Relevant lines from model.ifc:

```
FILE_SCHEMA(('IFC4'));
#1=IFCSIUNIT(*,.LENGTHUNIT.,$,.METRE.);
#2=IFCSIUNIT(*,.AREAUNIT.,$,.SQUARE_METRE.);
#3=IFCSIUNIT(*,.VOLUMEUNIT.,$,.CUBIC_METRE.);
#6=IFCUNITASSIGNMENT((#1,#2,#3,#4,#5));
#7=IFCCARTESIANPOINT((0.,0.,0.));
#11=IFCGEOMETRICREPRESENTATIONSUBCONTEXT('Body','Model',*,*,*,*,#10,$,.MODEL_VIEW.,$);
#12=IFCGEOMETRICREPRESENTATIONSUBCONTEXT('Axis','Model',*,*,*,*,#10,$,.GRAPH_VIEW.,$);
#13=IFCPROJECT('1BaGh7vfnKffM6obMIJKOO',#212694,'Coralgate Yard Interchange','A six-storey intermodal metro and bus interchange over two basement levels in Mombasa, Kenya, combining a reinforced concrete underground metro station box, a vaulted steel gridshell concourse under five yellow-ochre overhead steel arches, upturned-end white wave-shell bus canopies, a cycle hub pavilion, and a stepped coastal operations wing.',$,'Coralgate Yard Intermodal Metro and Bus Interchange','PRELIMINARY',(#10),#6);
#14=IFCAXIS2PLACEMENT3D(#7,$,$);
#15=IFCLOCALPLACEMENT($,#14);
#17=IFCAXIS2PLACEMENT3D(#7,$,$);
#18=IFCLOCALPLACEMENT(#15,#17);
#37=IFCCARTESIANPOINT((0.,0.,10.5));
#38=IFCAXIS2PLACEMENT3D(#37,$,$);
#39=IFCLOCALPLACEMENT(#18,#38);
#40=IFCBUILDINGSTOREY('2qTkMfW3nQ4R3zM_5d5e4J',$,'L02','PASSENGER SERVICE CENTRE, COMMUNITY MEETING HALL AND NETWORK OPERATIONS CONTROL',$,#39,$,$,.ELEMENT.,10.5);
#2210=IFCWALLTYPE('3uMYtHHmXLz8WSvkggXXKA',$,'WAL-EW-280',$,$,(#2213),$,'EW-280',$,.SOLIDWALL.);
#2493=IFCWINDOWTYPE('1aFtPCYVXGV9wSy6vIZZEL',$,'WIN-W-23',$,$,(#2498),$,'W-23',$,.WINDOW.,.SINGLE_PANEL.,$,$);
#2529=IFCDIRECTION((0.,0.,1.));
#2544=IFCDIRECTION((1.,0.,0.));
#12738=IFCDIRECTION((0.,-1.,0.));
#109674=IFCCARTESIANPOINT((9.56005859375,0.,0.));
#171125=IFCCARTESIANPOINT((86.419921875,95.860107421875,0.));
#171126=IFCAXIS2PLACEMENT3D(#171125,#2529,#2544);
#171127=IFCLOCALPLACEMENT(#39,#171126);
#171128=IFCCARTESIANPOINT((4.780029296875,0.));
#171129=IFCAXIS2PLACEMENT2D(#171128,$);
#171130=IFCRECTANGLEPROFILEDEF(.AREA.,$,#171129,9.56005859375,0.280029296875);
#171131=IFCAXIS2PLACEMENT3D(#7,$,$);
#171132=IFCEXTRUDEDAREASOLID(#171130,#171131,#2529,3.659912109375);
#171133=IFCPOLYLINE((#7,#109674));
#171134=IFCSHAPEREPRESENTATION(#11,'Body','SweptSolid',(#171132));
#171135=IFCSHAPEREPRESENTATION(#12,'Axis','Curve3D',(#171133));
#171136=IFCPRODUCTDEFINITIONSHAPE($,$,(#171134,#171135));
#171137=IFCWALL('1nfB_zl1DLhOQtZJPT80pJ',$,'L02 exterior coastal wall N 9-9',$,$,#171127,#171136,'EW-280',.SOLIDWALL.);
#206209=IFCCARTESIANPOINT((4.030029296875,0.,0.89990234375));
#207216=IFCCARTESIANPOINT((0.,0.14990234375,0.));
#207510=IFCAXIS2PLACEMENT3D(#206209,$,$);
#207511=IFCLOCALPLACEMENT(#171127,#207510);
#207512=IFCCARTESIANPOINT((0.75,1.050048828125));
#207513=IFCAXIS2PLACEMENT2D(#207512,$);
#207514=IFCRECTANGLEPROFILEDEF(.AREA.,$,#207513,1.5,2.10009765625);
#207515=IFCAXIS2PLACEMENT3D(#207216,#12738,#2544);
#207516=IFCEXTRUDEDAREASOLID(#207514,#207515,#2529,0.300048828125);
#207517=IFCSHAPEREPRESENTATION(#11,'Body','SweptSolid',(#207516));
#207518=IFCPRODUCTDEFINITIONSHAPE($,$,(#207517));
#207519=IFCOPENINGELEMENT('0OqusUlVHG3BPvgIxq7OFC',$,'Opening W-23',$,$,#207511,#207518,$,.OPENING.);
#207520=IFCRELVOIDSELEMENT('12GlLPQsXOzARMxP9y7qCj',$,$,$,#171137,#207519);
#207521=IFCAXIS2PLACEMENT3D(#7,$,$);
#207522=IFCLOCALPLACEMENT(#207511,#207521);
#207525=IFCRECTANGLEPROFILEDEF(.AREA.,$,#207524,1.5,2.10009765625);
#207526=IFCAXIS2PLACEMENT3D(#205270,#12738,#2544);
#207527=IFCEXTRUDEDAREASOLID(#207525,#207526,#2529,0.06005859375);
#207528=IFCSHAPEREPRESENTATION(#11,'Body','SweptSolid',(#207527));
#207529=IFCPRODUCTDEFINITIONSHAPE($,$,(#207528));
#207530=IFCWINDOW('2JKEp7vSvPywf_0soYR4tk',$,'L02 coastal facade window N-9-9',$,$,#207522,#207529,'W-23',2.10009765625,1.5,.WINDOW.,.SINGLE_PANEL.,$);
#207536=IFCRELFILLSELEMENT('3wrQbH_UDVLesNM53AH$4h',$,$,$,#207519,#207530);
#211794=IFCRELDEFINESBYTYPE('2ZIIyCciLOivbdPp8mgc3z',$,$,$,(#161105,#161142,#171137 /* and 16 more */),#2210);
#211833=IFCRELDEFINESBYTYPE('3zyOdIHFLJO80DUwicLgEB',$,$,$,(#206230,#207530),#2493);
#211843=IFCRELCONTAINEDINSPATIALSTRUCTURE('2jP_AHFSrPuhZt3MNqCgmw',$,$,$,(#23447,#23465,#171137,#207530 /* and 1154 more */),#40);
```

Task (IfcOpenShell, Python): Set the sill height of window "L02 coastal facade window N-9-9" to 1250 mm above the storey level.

```python
import numpy as np
import ifcopenshell
import ifcopenshell.api.geometry
import ifcopenshell.geom
import ifcopenshell.util.element
import ifcopenshell.util.placement
import ifcopenshell.util.shape
import ifcopenshell.util.unit

model = ifcopenshell.open("model.ifc")
unit_scale = ifcopenshell.util.unit.calculate_unit_scale(model)

window = model.by_guid("2JKEp7vSvPywf_0soYR4tk")
opening = window.FillsVoids[0].RelatingOpeningElement
storey = ifcopenshell.util.element.get_container(window, ifc_class="IfcBuildingStorey")
level = ifcopenshell.util.placement.get_local_placement(storey.ObjectPlacement)[2, 3]

# The opening's origin need not be at the sill, so measure its lowest point.
shape = ifcopenshell.geom.create_shape(ifcopenshell.geom.settings(), opening)
bottom = ifcopenshell.util.shape.get_shape_bottom_elevation(shape, shape.geometry) / unit_scale
dz = level + 1.25 / unit_scale - bottom

shift = np.array([0.0, 0.0, dz])
# The window is placed relative to its opening, so it follows when the opening moves.
matrix = ifcopenshell.util.placement.get_local_placement(opening.ObjectPlacement)
matrix[:3, 3] += shift
ifcopenshell.api.geometry.edit_object_placement(
    model, product=opening, matrix=matrix, is_si=False, should_transform_children=True
)

print(f"moved by {dz * unit_scale:+.3f} m")

model.write("model_rev.ifc")
```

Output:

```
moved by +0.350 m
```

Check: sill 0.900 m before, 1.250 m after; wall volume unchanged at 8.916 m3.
